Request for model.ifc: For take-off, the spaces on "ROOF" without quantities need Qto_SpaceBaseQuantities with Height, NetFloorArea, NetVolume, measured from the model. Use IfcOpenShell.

First a look at what the model holds.

```python
import ifcopenshell
import ifcopenshell.util.element
import ifcopenshell.util.unit

model = ifcopenshell.open("model.ifc")
print(model.schema)
for unit_type in ("LENGTHUNIT", "AREAUNIT", "VOLUMEUNIT"):
    print(unit_type, ifcopenshell.util.unit.calculate_unit_scale(model, unit_type))
storey = next(s for s in model.by_type("IfcBuildingStorey") if s.Name == "ROOF")
spaces = [e for e in ifcopenshell.util.element.get_decomposition(storey) if e.is_a("IfcSpace")]
for e in sorted(spaces, key=lambda e: e.id()):
    print(e.id(), e.is_a(), e.Name, list(ifcopenshell.util.element.get_psets(e, qtos_only=True)), sep=" | ")
```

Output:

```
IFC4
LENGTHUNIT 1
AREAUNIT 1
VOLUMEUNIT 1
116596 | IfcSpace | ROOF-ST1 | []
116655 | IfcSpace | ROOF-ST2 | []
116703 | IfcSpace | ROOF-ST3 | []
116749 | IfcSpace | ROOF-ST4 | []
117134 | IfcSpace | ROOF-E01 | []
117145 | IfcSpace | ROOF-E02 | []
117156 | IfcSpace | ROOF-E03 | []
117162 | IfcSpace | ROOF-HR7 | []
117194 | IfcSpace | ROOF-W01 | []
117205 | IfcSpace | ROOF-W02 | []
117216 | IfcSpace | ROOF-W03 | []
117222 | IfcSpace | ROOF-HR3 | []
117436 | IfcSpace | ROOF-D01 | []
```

```python
import ifcopenshell
import ifcopenshell.api.pset
import ifcopenshell.geom
import ifcopenshell.util.element
import ifcopenshell.util.shape
import ifcopenshell.util.unit

model = ifcopenshell.open("model.ifc")
unit_scale = ifcopenshell.util.unit.calculate_unit_scale(model)
area_scale = ifcopenshell.util.unit.calculate_unit_scale(model, "AREAUNIT")
volume_scale = ifcopenshell.util.unit.calculate_unit_scale(model, "VOLUMEUNIT")
settings = ifcopenshell.geom.settings()

storey = next(s for s in model.by_type("IfcBuildingStorey") if s.Name == "ROOF")
spaces = [e for e in ifcopenshell.util.element.get_decomposition(storey) if e.is_a("IfcSpace")]

for e in sorted(spaces, key=lambda e: e.id()):
    if ifcopenshell.util.element.get_psets(e, qtos_only=True, should_inherit=False):
        continue
    # Geometry comes back in metres, in the element's own axes.
    shape = ifcopenshell.geom.create_shape(settings, e)
    values = {
        "Height": ifcopenshell.util.shape.get_z(shape.geometry) / unit_scale,
        "NetFloorArea": ifcopenshell.util.shape.get_footprint_area(shape.geometry) / area_scale,
        "NetVolume": ifcopenshell.util.shape.get_volume(shape.geometry) / volume_scale,
    }
    qto = ifcopenshell.api.pset.add_qto(model, product=e, name="Qto_SpaceBaseQuantities")
    ifcopenshell.api.pset.edit_qto(model, qto=qto, properties=values)
    print(e.id(), {k: round(v, 3) for k, v in values.items()})

model.write("model_edited.ifc")
```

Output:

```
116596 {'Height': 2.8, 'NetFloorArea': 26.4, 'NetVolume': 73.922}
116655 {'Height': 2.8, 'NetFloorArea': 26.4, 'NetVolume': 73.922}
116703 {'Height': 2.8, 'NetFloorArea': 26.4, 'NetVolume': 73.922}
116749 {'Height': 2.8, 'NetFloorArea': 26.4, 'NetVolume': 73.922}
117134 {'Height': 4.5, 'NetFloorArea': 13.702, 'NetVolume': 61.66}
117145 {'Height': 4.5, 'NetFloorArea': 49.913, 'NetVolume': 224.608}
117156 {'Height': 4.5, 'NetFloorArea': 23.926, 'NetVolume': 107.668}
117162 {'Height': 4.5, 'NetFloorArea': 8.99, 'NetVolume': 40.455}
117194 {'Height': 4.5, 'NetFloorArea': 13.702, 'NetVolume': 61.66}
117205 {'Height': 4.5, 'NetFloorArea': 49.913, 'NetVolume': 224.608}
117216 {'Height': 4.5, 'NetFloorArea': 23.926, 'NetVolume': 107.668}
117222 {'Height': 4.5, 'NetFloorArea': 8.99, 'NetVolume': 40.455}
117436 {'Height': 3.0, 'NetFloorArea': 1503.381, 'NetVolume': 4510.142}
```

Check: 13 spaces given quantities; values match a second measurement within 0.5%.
